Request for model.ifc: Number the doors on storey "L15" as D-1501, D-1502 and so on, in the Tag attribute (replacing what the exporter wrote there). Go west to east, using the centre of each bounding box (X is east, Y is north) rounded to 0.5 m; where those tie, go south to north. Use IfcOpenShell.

First a look at what the model holds.

```python
import ifcopenshell
import ifcopenshell.util.element
import ifcopenshell.util.placement

model = ifcopenshell.open("model.ifc")
print(model.schema)
storey = next(s for s in model.by_type("IfcBuildingStorey") if s.Name == "L15")
doors = [e for e in ifcopenshell.util.element.get_decomposition(storey) if e.is_a("IfcDoor")]
for e in sorted(doors, key=lambda e: e.id()):
    origin = ifcopenshell.util.placement.get_local_placement(e.ObjectPlacement)[:3, 3]
    print(e.id(), e.Tag, e.Name, origin.round(2) + 0.0, sep=" | ")
```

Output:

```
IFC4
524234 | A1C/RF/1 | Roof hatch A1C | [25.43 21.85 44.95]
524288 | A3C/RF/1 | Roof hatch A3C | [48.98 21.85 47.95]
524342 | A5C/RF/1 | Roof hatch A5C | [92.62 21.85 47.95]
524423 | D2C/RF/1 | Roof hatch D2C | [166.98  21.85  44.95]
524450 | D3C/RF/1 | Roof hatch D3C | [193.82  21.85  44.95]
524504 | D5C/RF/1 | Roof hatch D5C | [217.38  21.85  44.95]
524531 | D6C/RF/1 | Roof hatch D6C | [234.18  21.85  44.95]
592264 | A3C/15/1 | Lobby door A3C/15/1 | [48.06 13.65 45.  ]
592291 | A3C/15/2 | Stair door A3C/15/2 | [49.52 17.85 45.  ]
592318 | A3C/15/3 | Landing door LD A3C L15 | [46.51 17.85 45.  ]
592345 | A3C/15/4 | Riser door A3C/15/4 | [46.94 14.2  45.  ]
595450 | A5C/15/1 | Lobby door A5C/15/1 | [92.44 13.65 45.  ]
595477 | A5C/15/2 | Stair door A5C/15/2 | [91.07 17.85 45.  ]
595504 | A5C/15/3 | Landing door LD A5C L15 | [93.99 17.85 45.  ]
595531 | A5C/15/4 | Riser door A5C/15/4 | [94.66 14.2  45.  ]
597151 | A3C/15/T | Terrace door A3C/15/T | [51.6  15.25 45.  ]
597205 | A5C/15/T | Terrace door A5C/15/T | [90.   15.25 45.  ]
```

```python
import ifcopenshell
import ifcopenshell.geom
import ifcopenshell.util.element
import ifcopenshell.util.shape

model = ifcopenshell.open("model.ifc")
settings = ifcopenshell.geom.settings()
settings.set("use-world-coords", True)


def centre(element):
    shape = ifcopenshell.geom.create_shape(settings, element)
    return ifcopenshell.util.shape.get_bbox_centroid(shape.geometry)


storey = next(s for s in model.by_type("IfcBuildingStorey") if s.Name == "L15")
doors = [e for e in ifcopenshell.util.element.get_decomposition(storey) if e.is_a("IfcDoor")]

# Insertion points can sit at a corner or the storey origin, so sort by the geometry (in metres).
centres = {e: centre(e) for e in doors}
doors.sort(key=lambda e: (round(centres[e][0] / 0.5), centres[e][1]))

for i, e in enumerate(doors, start=1):
    number = f"D-15{i:02d}"
    e.Tag = number
    print(e.id(), number)

model.write("model-out.ifc")
```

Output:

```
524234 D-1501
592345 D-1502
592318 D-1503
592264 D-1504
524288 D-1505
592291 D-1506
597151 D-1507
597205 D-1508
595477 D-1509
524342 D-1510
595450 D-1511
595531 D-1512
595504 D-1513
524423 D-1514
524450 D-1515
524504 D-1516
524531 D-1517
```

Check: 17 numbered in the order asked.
